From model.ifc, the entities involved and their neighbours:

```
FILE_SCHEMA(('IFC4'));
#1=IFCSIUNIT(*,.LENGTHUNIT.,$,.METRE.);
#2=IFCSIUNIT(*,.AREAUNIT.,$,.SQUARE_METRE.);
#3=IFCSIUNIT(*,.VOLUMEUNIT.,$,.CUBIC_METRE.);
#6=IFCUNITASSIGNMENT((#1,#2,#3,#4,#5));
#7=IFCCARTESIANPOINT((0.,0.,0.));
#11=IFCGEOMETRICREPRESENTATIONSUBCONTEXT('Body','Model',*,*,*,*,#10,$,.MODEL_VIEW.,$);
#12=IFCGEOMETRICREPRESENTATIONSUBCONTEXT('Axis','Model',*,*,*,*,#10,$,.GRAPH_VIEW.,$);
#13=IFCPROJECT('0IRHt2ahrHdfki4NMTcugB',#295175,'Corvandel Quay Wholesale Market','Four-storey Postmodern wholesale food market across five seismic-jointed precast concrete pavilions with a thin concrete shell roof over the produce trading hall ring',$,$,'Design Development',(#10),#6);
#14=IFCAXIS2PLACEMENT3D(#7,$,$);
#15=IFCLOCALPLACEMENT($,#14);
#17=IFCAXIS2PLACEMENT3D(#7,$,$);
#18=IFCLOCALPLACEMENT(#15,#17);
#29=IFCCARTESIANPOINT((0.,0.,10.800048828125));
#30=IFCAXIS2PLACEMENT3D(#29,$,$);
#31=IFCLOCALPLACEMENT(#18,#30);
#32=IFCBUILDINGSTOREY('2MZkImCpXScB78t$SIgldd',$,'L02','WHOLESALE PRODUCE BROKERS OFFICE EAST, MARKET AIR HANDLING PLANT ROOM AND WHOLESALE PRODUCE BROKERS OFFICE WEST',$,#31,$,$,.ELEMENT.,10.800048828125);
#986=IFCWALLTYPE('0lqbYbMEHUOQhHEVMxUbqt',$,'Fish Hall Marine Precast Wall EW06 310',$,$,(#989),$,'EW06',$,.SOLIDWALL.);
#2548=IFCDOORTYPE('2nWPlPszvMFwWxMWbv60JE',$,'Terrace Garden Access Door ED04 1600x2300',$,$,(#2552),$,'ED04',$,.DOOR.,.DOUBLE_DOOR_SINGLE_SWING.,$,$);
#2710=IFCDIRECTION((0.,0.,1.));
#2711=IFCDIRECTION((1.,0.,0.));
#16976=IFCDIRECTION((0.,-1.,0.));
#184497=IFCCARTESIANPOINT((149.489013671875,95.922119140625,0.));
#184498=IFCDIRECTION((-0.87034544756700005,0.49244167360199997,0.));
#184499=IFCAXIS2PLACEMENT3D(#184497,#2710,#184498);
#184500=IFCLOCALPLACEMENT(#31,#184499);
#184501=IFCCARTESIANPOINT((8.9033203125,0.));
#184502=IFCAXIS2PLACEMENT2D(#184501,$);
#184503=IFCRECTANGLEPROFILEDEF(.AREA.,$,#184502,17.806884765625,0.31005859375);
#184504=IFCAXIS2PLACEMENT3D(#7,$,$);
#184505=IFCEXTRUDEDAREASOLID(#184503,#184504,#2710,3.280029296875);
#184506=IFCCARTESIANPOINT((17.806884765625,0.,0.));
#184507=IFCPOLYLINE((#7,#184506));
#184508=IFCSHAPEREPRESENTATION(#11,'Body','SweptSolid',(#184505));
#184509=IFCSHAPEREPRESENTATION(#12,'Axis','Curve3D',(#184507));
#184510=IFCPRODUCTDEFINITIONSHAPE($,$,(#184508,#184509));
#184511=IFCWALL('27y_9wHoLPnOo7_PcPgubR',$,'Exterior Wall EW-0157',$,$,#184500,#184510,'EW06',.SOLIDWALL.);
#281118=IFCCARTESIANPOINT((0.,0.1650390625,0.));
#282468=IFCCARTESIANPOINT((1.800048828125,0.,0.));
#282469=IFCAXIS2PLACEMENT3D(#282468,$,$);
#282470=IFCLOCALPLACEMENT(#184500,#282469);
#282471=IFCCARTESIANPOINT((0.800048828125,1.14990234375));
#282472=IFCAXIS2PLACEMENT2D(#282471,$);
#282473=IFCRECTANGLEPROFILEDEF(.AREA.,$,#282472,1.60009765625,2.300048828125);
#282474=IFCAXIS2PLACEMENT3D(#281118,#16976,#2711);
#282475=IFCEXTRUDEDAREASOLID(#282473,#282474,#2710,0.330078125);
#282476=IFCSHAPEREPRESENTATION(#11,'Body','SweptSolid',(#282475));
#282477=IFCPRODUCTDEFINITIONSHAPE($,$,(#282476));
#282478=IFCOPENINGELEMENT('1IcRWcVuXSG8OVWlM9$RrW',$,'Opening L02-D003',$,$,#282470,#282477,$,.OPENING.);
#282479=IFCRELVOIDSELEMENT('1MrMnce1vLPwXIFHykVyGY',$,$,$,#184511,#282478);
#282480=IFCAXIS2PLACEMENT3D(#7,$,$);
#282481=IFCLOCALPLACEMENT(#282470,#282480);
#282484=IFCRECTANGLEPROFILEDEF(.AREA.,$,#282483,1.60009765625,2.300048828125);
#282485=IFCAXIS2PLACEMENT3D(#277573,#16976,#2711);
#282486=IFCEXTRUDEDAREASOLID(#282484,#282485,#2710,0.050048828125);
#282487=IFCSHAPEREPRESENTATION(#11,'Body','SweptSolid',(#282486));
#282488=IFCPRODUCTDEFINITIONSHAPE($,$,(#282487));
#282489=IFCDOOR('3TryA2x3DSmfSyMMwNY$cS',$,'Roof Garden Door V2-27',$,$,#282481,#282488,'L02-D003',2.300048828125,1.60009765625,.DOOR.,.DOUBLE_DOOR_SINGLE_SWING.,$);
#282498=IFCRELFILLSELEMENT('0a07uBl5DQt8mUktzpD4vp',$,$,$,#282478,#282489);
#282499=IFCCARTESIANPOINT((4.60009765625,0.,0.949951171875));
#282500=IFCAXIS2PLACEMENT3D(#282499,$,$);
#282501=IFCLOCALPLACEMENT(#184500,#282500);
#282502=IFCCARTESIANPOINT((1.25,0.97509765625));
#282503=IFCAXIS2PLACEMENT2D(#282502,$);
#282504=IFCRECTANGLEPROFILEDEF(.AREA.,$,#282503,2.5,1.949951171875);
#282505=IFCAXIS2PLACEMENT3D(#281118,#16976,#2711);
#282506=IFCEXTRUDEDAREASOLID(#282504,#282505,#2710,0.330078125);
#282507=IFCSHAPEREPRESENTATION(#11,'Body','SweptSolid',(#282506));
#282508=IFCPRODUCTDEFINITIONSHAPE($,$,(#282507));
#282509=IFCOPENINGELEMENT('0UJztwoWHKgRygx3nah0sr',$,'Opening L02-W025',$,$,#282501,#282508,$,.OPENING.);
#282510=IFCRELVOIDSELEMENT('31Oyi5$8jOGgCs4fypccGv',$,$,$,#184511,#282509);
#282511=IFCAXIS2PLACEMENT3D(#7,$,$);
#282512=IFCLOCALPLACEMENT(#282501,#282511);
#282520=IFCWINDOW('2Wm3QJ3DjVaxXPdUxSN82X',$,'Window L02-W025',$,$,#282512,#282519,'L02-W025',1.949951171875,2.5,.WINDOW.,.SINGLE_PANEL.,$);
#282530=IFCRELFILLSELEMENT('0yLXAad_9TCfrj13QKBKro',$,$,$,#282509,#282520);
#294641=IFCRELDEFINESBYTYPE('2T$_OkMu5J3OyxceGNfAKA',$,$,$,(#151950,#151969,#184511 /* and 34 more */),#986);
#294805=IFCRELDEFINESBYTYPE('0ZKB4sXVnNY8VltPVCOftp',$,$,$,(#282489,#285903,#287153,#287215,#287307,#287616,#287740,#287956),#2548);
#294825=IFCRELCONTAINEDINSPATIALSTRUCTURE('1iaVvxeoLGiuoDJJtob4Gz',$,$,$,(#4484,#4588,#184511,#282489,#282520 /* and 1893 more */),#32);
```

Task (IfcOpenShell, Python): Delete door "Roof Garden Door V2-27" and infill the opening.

```python
import ifcopenshell
import ifcopenshell.api.feature
import ifcopenshell.api.root
import ifcopenshell.geom
import ifcopenshell.util.shape

model = ifcopenshell.open("model.ifc")
settings = ifcopenshell.geom.settings()


def volume(element):
    """Net volume in cubic metres, openings subtracted."""
    shape = ifcopenshell.geom.create_shape(settings, element)
    return ifcopenshell.util.shape.get_volume(shape.geometry)


door = model.by_id(282489)
opening = door.FillsVoids[0].RelatingOpeningElement
wall = opening.VoidsElements[0].RelatingBuildingElement
before = volume(wall)

ifcopenshell.api.root.remove_product(model, product=door)
ifcopenshell.api.feature.remove_feature(model, feature=opening)

after = volume(wall)

print(f"wall volume {before:.3f} -> {after:.3f} m3")

model.write("model_v2.ifc")
```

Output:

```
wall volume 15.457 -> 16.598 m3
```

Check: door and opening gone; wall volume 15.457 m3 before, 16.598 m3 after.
